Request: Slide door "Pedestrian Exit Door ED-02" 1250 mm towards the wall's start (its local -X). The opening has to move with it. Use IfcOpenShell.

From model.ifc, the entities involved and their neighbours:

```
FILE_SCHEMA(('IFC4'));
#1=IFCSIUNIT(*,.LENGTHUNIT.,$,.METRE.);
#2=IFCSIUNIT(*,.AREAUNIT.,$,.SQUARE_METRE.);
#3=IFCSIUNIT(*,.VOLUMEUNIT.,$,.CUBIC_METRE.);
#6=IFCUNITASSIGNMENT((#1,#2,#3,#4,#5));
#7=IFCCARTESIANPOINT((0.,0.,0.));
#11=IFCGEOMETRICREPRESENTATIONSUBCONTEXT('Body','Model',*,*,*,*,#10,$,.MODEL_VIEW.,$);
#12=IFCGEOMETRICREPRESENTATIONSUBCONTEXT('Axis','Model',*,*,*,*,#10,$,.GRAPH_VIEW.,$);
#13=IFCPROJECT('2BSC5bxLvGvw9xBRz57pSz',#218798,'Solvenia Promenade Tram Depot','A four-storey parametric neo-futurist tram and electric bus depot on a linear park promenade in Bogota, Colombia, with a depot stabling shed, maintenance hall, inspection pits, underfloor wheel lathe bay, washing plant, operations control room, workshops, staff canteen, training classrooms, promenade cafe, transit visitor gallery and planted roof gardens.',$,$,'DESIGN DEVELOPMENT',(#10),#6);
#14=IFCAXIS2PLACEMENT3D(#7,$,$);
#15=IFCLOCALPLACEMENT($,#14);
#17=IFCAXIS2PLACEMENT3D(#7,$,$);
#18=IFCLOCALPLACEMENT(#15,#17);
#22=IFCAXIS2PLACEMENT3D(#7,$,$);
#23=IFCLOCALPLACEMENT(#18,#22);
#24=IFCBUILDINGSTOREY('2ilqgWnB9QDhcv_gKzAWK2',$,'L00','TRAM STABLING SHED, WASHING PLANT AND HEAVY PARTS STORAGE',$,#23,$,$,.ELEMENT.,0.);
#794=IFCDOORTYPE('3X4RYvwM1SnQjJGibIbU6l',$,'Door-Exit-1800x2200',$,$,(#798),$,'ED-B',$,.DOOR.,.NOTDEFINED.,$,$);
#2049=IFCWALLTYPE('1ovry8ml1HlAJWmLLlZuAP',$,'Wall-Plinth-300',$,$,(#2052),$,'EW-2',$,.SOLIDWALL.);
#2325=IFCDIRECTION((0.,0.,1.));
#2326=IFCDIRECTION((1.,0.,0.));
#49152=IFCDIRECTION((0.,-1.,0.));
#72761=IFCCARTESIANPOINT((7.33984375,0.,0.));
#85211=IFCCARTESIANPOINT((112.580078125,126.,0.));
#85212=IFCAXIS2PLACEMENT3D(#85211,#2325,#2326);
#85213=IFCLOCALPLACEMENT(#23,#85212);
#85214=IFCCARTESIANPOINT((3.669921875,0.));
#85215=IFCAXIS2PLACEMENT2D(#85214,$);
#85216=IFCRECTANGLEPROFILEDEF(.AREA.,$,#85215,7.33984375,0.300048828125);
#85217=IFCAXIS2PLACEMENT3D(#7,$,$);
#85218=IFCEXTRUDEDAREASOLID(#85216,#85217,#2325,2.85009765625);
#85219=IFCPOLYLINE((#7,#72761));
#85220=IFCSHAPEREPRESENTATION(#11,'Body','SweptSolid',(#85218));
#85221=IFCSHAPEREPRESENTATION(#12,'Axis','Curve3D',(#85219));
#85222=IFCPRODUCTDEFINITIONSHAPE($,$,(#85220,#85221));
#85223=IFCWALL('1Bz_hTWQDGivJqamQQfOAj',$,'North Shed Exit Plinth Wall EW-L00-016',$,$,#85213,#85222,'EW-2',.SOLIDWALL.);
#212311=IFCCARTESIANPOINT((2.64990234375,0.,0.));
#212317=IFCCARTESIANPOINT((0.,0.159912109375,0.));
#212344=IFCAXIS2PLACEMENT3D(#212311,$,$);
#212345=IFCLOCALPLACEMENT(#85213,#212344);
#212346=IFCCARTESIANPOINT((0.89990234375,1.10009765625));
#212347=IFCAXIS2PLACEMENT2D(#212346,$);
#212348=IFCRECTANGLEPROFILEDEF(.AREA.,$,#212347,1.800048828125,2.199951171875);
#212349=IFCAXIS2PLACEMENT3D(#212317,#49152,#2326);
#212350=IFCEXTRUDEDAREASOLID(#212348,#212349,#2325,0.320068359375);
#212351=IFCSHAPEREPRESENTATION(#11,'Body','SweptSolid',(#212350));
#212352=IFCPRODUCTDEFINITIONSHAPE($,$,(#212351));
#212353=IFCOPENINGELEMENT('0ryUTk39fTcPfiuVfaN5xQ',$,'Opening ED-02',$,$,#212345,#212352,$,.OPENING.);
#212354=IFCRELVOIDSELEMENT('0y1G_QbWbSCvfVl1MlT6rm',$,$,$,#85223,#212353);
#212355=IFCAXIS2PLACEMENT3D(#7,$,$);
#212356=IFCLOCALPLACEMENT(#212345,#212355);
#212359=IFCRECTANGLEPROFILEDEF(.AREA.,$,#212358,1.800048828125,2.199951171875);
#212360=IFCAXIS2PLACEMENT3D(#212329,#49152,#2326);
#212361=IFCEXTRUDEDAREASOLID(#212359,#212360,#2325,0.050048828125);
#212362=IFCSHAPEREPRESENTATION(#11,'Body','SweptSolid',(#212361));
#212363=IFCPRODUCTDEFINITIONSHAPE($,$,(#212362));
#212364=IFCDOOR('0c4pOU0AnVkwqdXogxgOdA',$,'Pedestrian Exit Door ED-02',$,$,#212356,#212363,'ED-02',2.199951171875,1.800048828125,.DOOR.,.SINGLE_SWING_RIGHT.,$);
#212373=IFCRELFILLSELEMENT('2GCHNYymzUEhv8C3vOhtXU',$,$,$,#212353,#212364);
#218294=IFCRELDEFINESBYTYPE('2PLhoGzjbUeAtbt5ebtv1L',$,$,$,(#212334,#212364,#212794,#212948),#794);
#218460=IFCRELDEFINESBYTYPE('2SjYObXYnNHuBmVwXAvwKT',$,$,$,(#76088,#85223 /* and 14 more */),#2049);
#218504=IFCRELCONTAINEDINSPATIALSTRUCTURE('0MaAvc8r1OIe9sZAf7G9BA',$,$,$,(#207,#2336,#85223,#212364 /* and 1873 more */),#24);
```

```python
import ifcopenshell
import ifcopenshell.api.geometry
import ifcopenshell.util.placement
import ifcopenshell.util.unit

model = ifcopenshell.open("model.ifc")
unit_scale = ifcopenshell.util.unit.calculate_unit_scale(model)

door = model.by_guid("0c4pOU0AnVkwqdXogxgOdA")
opening = door.FillsVoids[0].RelatingOpeningElement
wall = opening.VoidsElements[0].RelatingBuildingElement

wall_matrix = ifcopenshell.util.placement.get_local_placement(wall.ObjectPlacement)
shift = wall_matrix[:3, 0] * -1.25 / unit_scale
before = ifcopenshell.util.placement.get_local_placement(door.ObjectPlacement)[:3, 3].copy()

# The door is placed relative to its opening, so it follows when the opening moves.
matrix = ifcopenshell.util.placement.get_local_placement(opening.ObjectPlacement)
matrix[:3, 3] += shift
ifcopenshell.api.geometry.edit_object_placement(
    model, product=opening, matrix=matrix, is_si=False, should_transform_children=True
)

after = ifcopenshell.util.placement.get_local_placement(door.ObjectPlacement)[:3, 3]
print("door moved by", (after - before).round(3) + 0.0)

model.write("model-out.ifc")
```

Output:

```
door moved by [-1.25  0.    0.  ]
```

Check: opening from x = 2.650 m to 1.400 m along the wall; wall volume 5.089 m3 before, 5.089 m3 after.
